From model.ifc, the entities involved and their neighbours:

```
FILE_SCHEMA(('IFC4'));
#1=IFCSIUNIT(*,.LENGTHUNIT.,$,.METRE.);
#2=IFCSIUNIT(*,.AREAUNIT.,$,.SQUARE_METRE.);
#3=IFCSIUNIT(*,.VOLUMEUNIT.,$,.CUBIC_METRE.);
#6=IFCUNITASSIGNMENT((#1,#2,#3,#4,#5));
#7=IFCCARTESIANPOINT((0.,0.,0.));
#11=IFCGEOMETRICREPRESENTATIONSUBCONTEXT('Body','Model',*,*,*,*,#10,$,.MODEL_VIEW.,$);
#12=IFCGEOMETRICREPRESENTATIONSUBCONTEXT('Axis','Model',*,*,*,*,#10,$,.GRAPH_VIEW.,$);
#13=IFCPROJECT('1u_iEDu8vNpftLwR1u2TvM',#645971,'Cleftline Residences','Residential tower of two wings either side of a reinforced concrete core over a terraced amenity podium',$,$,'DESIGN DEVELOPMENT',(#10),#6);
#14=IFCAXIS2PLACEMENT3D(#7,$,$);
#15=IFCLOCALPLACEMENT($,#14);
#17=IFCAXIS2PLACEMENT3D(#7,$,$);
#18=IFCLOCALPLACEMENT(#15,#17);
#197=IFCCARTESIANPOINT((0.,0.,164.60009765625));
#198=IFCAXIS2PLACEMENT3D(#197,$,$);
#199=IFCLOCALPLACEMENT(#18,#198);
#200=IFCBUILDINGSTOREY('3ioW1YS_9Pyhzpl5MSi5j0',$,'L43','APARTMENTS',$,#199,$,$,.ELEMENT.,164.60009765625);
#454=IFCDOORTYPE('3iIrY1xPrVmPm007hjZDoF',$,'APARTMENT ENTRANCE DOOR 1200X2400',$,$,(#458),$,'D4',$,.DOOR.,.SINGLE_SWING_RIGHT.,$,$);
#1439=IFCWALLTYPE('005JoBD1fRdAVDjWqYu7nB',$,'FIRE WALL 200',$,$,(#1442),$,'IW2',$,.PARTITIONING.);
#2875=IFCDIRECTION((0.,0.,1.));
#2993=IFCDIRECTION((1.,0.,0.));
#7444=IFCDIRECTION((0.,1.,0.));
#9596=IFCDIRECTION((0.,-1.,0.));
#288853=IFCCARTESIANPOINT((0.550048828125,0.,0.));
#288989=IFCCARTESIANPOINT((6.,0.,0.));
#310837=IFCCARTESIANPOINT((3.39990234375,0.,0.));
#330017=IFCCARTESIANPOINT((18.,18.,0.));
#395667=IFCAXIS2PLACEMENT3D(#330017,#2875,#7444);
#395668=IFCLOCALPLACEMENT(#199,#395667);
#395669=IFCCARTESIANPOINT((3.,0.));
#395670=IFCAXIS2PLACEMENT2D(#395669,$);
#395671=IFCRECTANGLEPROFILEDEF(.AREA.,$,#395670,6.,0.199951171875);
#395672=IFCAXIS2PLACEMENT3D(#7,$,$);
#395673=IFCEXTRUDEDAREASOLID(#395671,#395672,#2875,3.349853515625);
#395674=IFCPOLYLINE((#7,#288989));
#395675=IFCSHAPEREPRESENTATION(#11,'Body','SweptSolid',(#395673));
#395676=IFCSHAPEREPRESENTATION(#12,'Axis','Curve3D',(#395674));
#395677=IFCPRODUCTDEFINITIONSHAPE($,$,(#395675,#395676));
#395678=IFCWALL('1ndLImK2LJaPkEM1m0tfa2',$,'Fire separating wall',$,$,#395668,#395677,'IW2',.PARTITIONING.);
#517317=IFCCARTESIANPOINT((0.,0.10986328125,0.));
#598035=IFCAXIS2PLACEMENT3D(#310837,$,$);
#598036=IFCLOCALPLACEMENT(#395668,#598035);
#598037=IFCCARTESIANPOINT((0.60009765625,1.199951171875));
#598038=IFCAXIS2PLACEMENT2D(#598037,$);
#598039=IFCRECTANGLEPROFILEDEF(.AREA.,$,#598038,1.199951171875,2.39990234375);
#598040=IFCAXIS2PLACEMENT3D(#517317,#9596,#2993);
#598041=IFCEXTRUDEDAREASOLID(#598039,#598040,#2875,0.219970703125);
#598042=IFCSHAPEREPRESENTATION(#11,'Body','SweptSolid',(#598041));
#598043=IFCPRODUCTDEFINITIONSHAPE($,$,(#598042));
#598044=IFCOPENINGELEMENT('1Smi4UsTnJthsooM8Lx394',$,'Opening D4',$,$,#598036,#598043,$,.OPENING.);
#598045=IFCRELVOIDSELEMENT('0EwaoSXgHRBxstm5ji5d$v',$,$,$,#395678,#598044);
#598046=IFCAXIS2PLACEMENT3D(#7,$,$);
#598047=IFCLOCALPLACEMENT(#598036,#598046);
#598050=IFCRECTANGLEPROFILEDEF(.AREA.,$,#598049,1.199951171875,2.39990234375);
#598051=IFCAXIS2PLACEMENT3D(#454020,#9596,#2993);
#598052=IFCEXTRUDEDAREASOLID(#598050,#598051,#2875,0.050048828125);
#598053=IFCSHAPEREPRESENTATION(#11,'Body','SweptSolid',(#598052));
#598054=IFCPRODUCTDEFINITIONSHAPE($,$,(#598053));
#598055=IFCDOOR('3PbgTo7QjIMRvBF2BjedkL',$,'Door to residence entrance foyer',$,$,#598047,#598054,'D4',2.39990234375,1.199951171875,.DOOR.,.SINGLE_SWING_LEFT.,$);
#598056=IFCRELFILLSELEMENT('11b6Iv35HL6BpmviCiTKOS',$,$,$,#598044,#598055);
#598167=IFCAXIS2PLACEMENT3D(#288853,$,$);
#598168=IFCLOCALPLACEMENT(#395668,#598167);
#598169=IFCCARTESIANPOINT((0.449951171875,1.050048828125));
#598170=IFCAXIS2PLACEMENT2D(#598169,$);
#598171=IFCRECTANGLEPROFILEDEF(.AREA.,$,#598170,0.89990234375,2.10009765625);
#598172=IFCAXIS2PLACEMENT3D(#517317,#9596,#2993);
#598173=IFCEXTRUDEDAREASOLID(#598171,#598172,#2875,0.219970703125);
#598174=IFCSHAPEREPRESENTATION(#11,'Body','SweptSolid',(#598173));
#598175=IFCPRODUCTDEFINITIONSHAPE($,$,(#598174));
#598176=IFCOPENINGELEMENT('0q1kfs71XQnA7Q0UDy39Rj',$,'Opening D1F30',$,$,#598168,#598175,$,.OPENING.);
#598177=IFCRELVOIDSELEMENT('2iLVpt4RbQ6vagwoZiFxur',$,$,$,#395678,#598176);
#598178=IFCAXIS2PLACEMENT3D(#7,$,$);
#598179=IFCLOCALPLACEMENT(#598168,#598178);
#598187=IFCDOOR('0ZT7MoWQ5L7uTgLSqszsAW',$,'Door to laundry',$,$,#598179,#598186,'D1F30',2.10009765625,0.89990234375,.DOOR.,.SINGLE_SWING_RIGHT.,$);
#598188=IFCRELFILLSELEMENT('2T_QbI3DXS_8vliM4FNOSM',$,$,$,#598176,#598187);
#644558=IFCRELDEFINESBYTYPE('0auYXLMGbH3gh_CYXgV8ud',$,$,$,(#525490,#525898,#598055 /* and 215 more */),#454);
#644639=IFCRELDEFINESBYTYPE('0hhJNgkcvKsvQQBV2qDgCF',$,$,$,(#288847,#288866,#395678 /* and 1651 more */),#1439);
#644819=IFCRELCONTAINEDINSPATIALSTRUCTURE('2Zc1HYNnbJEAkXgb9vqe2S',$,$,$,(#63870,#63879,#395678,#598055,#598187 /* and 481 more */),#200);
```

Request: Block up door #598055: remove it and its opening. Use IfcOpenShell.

```python
import ifcopenshell
import ifcopenshell.api.feature
import ifcopenshell.api.root
import ifcopenshell.geom
import ifcopenshell.util.shape

model = ifcopenshell.open("model.ifc")
settings = ifcopenshell.geom.settings()


def volume(element):
    """Net volume in cubic metres, openings subtracted."""
    shape = ifcopenshell.geom.create_shape(settings, element)
    return ifcopenshell.util.shape.get_volume(shape.geometry)


door = model.by_guid("3PbgTo7QjIMRvBF2BjedkL")
opening = door.FillsVoids[0].RelatingOpeningElement
wall = opening.VoidsElements[0].RelatingBuildingElement
before = volume(wall)

ifcopenshell.api.root.remove_product(model, product=door)
ifcopenshell.api.feature.remove_feature(model, feature=opening)

after = volume(wall)

print(f"wall volume {before:.3f} -> {after:.3f} m3")

model.write("model_updated.ifc")
```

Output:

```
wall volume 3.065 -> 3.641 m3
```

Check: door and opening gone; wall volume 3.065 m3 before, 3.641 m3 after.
